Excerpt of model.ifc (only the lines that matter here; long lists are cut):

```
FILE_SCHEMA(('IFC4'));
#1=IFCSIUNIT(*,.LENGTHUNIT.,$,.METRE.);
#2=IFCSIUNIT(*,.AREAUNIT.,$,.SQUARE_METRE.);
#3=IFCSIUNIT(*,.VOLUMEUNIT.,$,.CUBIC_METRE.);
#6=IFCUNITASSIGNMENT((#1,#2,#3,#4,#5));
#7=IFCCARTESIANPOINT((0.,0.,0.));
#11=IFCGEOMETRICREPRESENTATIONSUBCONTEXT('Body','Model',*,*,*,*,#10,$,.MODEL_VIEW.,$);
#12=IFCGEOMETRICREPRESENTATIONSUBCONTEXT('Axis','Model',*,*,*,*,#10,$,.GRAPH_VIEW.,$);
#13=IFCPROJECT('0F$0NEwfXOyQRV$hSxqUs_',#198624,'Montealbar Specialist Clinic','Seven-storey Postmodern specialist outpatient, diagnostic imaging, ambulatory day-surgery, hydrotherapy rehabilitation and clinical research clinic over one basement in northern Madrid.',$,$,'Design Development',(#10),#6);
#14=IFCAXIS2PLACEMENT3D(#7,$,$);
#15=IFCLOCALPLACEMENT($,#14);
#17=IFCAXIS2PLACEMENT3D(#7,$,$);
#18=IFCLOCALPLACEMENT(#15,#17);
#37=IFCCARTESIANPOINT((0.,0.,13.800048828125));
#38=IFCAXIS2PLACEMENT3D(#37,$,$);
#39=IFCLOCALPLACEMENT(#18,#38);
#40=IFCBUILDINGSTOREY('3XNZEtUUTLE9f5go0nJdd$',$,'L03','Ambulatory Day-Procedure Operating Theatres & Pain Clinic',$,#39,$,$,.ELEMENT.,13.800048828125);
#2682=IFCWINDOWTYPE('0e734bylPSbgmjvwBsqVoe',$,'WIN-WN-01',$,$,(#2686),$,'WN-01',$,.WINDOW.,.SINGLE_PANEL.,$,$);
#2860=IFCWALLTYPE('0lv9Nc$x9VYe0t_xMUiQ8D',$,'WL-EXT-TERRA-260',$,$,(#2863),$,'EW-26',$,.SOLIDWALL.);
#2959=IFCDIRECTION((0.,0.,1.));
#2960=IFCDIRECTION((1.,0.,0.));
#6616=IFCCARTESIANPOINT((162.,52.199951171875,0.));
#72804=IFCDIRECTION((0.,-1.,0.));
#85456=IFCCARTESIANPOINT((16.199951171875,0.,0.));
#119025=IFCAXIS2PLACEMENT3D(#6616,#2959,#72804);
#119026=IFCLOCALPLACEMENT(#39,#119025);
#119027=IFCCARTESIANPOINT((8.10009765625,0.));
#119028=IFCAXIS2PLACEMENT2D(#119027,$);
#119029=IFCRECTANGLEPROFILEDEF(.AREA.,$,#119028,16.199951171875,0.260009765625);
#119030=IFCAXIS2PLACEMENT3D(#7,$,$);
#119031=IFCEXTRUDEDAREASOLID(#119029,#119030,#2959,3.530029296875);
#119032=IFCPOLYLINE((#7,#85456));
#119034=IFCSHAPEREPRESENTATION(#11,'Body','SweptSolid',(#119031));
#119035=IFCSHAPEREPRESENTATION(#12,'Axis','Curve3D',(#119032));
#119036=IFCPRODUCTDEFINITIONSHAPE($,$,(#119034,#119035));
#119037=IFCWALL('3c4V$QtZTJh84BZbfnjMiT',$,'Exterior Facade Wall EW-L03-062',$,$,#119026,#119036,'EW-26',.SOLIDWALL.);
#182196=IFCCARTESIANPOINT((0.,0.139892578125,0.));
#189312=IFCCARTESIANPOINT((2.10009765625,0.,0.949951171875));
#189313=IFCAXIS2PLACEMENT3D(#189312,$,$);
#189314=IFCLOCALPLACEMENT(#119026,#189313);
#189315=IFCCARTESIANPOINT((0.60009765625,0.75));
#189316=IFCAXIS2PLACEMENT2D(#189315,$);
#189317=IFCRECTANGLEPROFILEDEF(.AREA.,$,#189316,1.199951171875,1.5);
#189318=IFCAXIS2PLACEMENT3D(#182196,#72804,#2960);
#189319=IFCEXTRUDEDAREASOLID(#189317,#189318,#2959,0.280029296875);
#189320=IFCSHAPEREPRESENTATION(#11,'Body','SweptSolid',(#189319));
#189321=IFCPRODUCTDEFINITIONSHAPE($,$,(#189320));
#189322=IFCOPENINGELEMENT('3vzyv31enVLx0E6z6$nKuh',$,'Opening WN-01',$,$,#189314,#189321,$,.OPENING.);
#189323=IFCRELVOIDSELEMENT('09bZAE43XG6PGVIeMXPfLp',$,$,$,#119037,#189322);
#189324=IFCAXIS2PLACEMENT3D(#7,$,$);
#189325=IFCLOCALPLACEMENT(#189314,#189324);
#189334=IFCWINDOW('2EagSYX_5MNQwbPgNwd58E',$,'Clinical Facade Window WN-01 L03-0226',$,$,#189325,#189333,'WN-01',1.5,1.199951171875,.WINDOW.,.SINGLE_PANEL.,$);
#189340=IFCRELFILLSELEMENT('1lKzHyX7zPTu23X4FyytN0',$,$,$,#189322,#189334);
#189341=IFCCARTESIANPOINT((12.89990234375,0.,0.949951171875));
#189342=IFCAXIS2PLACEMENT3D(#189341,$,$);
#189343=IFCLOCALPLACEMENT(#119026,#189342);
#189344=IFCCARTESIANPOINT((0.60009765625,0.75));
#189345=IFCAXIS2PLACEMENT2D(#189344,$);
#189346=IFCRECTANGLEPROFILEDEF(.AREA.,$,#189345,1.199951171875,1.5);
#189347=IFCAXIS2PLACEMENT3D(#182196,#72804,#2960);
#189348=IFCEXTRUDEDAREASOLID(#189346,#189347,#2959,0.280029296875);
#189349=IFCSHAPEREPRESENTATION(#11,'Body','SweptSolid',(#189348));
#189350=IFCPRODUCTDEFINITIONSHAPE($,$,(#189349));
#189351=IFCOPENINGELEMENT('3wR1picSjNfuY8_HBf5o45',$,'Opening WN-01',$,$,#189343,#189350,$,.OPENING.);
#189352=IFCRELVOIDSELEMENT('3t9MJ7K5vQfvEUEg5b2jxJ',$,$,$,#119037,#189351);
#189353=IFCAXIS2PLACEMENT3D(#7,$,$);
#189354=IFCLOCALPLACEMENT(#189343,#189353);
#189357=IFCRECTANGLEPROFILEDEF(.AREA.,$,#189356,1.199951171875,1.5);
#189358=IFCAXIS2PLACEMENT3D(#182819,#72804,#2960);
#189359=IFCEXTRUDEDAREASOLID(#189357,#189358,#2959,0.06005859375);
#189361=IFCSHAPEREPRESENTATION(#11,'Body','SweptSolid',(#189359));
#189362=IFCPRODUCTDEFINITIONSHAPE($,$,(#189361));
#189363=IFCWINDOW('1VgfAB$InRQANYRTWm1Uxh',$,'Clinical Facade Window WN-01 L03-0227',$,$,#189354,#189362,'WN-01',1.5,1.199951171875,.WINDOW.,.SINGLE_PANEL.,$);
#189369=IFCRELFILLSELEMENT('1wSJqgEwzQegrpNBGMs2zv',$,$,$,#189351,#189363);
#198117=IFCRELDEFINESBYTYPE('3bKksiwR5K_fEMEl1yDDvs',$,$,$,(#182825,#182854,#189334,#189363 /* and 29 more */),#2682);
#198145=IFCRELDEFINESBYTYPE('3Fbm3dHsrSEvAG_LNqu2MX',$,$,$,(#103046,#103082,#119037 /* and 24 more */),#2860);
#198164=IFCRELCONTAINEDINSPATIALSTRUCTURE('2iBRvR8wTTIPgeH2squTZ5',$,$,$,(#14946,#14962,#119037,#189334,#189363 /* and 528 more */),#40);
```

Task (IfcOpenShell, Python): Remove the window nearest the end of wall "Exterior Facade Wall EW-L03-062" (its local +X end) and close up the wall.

```python
import ifcopenshell
import ifcopenshell.api.feature
import ifcopenshell.api.root
import ifcopenshell.geom
import ifcopenshell.util.shape

model = ifcopenshell.open("model.ifc")
settings = ifcopenshell.geom.settings()


def volume(element):
    """Net volume in cubic metres, openings subtracted."""
    shape = ifcopenshell.geom.create_shape(settings, element)
    return ifcopenshell.util.shape.get_volume(shape.geometry)


window = model.by_guid("1VgfAB$InRQANYRTWm1Uxh")
opening = window.FillsVoids[0].RelatingOpeningElement
wall = opening.VoidsElements[0].RelatingBuildingElement
before = volume(wall)

ifcopenshell.api.root.remove_product(model, product=window)
ifcopenshell.api.feature.remove_feature(model, feature=opening)

after = volume(wall)

print(f"wall volume {before:.3f} -> {after:.3f} m3")

model.write("model_edited.ifc")
```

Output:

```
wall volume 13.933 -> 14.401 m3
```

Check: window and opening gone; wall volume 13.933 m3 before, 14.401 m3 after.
